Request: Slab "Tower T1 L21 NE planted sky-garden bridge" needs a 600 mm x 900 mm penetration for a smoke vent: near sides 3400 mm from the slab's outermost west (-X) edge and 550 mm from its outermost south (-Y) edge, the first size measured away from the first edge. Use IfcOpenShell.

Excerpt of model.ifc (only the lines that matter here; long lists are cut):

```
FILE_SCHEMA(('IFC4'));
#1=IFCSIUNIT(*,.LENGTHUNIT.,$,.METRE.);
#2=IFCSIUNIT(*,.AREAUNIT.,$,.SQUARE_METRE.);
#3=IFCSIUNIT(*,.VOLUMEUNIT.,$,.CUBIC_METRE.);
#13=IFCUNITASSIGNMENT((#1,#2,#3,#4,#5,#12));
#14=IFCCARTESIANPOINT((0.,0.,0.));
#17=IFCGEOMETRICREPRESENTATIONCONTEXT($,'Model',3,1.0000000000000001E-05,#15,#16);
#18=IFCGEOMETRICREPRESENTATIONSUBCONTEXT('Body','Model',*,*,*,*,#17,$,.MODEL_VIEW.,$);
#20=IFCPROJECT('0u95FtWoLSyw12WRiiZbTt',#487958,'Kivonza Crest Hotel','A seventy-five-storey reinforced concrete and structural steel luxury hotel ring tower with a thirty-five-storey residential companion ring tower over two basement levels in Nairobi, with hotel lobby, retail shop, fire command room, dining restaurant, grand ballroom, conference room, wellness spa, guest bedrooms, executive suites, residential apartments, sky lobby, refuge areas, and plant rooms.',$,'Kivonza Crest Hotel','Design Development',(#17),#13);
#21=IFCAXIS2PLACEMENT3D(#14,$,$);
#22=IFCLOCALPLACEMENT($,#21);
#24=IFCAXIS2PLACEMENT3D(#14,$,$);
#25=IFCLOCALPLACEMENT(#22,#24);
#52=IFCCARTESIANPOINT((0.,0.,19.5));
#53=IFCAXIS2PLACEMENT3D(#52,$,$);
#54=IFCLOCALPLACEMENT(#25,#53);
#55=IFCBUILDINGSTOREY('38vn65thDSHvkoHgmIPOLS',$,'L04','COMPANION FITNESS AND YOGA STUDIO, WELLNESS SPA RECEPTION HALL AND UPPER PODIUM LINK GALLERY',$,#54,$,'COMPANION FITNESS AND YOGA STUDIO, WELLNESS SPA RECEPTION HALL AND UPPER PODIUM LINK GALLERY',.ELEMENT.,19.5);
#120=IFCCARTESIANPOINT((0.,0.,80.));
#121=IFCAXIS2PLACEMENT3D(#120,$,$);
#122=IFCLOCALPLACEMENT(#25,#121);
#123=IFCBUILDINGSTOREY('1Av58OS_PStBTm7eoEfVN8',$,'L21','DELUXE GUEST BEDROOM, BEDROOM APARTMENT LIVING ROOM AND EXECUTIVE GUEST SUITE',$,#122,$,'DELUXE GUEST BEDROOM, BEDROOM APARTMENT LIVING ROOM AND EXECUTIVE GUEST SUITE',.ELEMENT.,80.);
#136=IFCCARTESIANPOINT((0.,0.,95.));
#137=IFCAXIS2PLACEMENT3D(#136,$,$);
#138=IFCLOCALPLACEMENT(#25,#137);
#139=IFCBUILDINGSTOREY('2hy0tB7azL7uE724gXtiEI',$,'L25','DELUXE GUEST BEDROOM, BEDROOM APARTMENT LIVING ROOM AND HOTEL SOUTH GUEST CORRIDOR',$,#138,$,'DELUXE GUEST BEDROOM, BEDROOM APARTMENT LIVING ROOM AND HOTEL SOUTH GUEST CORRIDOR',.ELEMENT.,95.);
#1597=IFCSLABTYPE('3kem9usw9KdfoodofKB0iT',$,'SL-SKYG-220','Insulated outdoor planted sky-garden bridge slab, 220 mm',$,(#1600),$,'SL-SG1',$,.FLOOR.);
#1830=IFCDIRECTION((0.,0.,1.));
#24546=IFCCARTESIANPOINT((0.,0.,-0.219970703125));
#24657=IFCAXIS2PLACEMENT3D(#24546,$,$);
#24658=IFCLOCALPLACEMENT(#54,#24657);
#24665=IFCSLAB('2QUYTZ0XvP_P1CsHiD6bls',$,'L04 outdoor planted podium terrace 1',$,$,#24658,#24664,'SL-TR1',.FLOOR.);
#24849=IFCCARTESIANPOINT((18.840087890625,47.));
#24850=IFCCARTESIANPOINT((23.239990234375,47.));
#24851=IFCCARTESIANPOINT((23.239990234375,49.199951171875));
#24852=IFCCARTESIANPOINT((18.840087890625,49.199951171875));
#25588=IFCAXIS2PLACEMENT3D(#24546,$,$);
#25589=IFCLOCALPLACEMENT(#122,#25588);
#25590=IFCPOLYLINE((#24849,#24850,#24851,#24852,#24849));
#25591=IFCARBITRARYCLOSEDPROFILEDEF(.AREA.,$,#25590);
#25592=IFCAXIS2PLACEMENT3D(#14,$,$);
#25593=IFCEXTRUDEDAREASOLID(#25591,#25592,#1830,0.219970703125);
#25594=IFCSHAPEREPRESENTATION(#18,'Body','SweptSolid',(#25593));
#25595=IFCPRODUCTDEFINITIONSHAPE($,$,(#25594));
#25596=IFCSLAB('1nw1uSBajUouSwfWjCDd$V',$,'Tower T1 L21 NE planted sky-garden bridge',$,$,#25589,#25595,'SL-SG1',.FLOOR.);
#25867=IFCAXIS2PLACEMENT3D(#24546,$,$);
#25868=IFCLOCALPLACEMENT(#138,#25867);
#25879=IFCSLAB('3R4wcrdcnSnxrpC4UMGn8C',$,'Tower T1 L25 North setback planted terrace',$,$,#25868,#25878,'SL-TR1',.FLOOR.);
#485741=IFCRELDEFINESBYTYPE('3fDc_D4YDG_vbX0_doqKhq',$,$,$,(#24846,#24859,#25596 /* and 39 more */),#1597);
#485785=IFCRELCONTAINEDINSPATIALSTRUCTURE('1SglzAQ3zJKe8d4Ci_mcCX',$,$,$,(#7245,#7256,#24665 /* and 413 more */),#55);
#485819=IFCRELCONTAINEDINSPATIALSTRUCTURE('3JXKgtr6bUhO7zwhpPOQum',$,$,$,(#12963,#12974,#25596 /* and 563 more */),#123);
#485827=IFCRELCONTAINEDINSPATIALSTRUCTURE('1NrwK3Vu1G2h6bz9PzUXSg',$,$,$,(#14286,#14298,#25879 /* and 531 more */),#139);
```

```python
import numpy as np
import ifcopenshell
import ifcopenshell.api.feature
import ifcopenshell.api.geometry
import ifcopenshell.api.root
import ifcopenshell.geom
import ifcopenshell.util.placement
import ifcopenshell.util.representation
import ifcopenshell.util.shape
import ifcopenshell.util.unit

model = ifcopenshell.open("model.ifc")
unit_scale = ifcopenshell.util.unit.calculate_unit_scale(model)
settings = ifcopenshell.geom.settings()


def volume(element):
    """Net volume in cubic metres, openings subtracted."""
    shape = ifcopenshell.geom.create_shape(settings, element)
    return ifcopenshell.util.shape.get_volume(shape.geometry)


slab = model.by_guid("1nw1uSBajUouSwfWjCDd$V")
before = volume(slab)

# Extent in the slab's own axes, in metres. The edges named are its -X and -Y sides.
slab_shape = ifcopenshell.geom.create_shape(settings, slab)
vertices = ifcopenshell.util.shape.get_vertices(slab_shape.geometry)
x_min, y_min, bottom = vertices.min(axis=0)
top = vertices[:, 2].max()

opening = ifcopenshell.api.root.create_entity(model, ifc_class="IfcOpeningElement", name="Smoke vent opening", predefined_type="OPENING")
context = ifcopenshell.util.representation.get_context(model, "Model", "Body", "MODEL_VIEW")
width, depth = 0.6, 0.9
outline = [(0.0, 0.0), (width, 0.0), (width, depth), (0.0, depth), (0.0, 0.0)]
# Overshoot both faces by 50 mm so the cut is clean.
shape = ifcopenshell.api.geometry.add_slab_representation(
    model, context=context, depth=top - bottom + 0.1, polyline=outline
)
ifcopenshell.api.geometry.assign_representation(model, product=opening, representation=shape)

matrix = ifcopenshell.util.placement.get_local_placement(slab.ObjectPlacement)
matrix[:, 3] = matrix @ np.append(np.array([x_min + 3.4, y_min + 0.55, bottom - 0.05]) / unit_scale, 1.0)
ifcopenshell.api.geometry.edit_object_placement(model, product=opening, matrix=matrix, is_si=False)
ifcopenshell.api.feature.add_feature(model, feature=opening, element=slab)

after = volume(slab)

print(f"slab volume {before:.3f} -> {after:.3f} m3")

model.write("model_edited.ifc")
```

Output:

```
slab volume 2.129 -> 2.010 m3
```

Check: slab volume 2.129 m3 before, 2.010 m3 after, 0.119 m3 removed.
